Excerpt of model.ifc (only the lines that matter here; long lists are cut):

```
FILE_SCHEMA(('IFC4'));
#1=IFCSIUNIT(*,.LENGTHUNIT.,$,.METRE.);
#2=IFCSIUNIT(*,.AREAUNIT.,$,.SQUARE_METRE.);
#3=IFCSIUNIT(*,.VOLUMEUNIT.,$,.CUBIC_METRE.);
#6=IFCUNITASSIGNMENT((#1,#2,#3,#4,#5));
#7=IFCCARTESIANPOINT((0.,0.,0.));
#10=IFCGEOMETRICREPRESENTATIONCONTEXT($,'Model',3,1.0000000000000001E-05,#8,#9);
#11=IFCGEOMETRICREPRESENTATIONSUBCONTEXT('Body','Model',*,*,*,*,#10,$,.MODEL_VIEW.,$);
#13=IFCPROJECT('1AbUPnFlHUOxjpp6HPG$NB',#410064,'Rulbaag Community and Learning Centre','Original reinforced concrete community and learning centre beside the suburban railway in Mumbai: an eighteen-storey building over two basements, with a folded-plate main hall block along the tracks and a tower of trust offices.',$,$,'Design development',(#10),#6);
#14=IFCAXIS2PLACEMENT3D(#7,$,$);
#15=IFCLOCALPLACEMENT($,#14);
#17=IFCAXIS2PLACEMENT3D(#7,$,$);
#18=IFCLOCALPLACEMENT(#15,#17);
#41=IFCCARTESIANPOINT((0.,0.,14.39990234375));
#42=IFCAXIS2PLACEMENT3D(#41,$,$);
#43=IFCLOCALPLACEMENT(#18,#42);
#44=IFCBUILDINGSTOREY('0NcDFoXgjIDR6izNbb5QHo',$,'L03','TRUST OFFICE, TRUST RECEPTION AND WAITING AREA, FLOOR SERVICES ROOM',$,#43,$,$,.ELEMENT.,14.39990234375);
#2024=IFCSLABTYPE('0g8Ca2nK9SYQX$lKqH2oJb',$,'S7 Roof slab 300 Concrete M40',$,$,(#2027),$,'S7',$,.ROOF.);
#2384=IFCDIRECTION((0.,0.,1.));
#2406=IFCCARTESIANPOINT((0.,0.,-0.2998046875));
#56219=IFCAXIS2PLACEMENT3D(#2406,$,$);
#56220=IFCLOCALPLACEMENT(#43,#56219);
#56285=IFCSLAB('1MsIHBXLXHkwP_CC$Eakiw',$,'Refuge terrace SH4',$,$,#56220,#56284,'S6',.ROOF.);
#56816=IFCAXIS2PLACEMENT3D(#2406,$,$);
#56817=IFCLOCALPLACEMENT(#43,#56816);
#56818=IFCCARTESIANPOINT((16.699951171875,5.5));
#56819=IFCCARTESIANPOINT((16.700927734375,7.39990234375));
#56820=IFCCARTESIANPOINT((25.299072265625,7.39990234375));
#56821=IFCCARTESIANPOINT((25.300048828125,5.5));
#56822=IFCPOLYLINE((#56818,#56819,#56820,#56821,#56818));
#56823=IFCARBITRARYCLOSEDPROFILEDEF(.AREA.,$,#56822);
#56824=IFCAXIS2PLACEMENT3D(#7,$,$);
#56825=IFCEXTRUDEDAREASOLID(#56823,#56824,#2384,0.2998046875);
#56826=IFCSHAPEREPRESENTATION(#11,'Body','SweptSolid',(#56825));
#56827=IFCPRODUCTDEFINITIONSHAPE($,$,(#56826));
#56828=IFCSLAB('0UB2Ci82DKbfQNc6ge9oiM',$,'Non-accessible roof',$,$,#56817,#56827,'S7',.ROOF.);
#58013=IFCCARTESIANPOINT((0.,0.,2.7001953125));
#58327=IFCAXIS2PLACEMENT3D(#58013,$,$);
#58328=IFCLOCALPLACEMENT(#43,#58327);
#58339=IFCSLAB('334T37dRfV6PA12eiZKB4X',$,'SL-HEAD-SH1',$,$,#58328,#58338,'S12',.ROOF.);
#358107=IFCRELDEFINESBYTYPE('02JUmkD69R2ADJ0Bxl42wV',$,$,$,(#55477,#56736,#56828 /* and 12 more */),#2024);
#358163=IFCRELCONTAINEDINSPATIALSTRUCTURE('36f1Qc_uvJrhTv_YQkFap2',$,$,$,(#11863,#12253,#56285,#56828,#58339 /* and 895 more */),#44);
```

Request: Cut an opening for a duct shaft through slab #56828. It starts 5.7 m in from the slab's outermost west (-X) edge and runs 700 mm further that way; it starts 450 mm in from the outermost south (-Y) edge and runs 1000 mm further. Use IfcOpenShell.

```python
import numpy as np
import ifcopenshell
import ifcopenshell.api.feature
import ifcopenshell.api.geometry
import ifcopenshell.api.root
import ifcopenshell.geom
import ifcopenshell.util.placement
import ifcopenshell.util.representation
import ifcopenshell.util.shape
import ifcopenshell.util.unit

model = ifcopenshell.open("model.ifc")
unit_scale = ifcopenshell.util.unit.calculate_unit_scale(model)
settings = ifcopenshell.geom.settings()


def volume(element):
    """Net volume in cubic metres, openings subtracted."""
    shape = ifcopenshell.geom.create_shape(settings, element)
    return ifcopenshell.util.shape.get_volume(shape.geometry)


slab = model.by_guid("0UB2Ci82DKbfQNc6ge9oiM")
before = volume(slab)

# Extent in the slab's own axes, in metres. The edges named are its -X and -Y sides.
slab_shape = ifcopenshell.geom.create_shape(settings, slab)
vertices = ifcopenshell.util.shape.get_vertices(slab_shape.geometry)
x_min, y_min, bottom = vertices.min(axis=0)
top = vertices[:, 2].max()

opening = ifcopenshell.api.root.create_entity(model, ifc_class="IfcOpeningElement", name="Duct shaft opening", predefined_type="OPENING")
context = ifcopenshell.util.representation.get_context(model, "Model", "Body", "MODEL_VIEW")
width, depth = 0.7, 1
outline = [(0.0, 0.0), (width, 0.0), (width, depth), (0.0, depth), (0.0, 0.0)]
# Overshoot both faces by 50 mm so the cut is clean.
shape = ifcopenshell.api.geometry.add_slab_representation(
    model, context=context, depth=top - bottom + 0.1, polyline=outline
)
ifcopenshell.api.geometry.assign_representation(model, product=opening, representation=shape)

matrix = ifcopenshell.util.placement.get_local_placement(slab.ObjectPlacement)
matrix[:, 3] = matrix @ np.append(np.array([x_min + 5.7, y_min + 0.45, bottom - 0.05]) / unit_scale, 1.0)
ifcopenshell.api.geometry.edit_object_placement(model, product=opening, matrix=matrix, is_si=False)
ifcopenshell.api.feature.add_feature(model, feature=opening, element=slab)

after = volume(slab)

print(f"slab volume {before:.3f} -> {after:.3f} m3")

model.write("model_rev.ifc")
```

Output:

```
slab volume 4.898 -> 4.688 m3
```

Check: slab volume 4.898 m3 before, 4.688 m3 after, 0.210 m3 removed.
